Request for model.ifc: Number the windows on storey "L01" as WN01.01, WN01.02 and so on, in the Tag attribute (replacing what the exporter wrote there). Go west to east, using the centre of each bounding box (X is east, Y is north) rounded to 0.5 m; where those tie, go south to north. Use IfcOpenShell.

First a look at what the model holds.

```python
import ifcopenshell
import ifcopenshell.util.element
import ifcopenshell.util.placement

model = ifcopenshell.open("model.ifc")
print(model.schema)
storey = next(s for s in model.by_type("IfcBuildingStorey") if s.Name == "L01")
windows = [e for e in ifcopenshell.util.element.get_decomposition(storey) if e.is_a("IfcWindow")]
for e in sorted(windows, key=lambda e: e.id()):
    origin = ifcopenshell.util.placement.get_local_placement(e.ObjectPlacement)[:3, 3]
    print(e.id(), e.Tag, e.Name, origin.round(2) + 0.0, sep=" | ")
```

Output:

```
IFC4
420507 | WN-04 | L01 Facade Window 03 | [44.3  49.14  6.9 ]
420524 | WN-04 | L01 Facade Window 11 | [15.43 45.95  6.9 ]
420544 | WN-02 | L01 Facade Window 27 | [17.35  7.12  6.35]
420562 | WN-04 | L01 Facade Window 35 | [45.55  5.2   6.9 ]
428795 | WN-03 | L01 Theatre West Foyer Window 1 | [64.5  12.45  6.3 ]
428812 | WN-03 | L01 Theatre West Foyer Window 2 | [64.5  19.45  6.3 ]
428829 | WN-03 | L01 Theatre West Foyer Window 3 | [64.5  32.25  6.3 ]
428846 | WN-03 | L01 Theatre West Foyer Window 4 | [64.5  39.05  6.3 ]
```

```python
import ifcopenshell
import ifcopenshell.geom
import ifcopenshell.util.element
import ifcopenshell.util.shape

model = ifcopenshell.open("model.ifc")
settings = ifcopenshell.geom.settings()
settings.set("use-world-coords", True)


def centre(element):
    shape = ifcopenshell.geom.create_shape(settings, element)
    return ifcopenshell.util.shape.get_bbox_centroid(shape.geometry)


storey = next(s for s in model.by_type("IfcBuildingStorey") if s.Name == "L01")
windows = [e for e in ifcopenshell.util.element.get_decomposition(storey) if e.is_a("IfcWindow")]

# Insertion points can sit at a corner or the storey origin, so sort by the geometry (in metres).
centres = {e: centre(e) for e in windows}
windows.sort(key=lambda e: (round(centres[e][0] / 0.5), centres[e][1]))

for i, e in enumerate(windows, start=1):
    number = f"WN01.{i:02d}"
    e.Tag = number
    print(e.id(), number)

model.write("model-out.ifc")
```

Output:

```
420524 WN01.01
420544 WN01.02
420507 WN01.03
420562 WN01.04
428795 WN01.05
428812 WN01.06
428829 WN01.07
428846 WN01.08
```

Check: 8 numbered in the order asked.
